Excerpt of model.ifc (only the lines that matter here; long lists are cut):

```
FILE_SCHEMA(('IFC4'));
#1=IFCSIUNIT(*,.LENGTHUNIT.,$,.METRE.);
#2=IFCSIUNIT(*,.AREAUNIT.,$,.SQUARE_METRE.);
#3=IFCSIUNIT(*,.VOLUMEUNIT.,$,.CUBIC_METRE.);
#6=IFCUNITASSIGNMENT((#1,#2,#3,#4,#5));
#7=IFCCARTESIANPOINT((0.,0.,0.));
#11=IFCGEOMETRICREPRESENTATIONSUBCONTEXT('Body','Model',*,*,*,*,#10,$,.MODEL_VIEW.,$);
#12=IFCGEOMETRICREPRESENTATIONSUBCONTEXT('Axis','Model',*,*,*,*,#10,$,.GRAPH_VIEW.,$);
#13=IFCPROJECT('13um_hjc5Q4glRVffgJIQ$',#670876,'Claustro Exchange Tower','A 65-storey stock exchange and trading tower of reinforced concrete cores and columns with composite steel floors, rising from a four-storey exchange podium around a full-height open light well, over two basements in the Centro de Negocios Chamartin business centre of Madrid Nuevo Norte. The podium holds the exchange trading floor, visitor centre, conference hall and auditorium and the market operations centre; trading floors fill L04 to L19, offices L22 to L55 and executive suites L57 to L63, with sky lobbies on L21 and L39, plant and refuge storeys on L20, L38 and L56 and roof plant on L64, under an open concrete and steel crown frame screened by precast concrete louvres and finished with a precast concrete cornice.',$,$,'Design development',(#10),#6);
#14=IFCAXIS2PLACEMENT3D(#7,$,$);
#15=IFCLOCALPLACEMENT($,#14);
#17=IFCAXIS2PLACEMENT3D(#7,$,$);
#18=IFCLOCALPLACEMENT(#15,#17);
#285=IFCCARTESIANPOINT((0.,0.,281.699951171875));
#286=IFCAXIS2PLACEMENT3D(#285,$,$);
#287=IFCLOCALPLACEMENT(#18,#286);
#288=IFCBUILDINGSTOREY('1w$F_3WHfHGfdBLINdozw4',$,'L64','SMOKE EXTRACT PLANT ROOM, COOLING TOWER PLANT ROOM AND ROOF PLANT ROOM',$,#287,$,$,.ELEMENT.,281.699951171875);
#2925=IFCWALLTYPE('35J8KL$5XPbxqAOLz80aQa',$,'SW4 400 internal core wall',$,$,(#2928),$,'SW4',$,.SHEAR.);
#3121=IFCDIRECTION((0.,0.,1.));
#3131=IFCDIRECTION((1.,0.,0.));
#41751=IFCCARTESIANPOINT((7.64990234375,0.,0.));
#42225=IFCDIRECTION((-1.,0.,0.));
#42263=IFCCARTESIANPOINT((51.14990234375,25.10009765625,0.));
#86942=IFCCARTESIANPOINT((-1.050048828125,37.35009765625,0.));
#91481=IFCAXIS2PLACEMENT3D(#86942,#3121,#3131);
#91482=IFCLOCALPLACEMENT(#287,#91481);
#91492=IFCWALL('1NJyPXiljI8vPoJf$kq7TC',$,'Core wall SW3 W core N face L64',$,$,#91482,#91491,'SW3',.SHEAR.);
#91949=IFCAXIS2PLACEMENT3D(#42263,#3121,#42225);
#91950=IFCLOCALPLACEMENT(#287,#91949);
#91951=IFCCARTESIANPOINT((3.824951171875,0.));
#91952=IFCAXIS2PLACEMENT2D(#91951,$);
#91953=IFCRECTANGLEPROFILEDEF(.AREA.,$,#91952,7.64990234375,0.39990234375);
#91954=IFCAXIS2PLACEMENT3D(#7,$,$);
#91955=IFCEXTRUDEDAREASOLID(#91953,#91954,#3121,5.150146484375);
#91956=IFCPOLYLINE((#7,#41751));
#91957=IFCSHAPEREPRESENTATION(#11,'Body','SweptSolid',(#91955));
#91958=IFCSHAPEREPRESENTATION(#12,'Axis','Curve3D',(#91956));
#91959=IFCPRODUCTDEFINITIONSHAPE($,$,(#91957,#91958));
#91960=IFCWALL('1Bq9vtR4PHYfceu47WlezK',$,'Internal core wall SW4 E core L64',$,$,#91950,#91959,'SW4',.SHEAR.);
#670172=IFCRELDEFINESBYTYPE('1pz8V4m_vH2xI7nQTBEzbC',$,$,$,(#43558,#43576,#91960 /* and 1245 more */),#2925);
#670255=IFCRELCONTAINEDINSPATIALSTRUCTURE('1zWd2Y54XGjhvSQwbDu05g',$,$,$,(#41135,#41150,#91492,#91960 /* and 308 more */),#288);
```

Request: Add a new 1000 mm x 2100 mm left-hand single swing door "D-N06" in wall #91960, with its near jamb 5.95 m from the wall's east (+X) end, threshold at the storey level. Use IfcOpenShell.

```python
import numpy as np
import ifcopenshell
import ifcopenshell.api.feature
import ifcopenshell.api.geometry
import ifcopenshell.api.root
import ifcopenshell.api.spatial
import ifcopenshell.geom
import ifcopenshell.util.element
import ifcopenshell.util.placement
import ifcopenshell.util.representation
import ifcopenshell.util.shape
import ifcopenshell.util.unit

model = ifcopenshell.open("model.ifc")
unit_scale = ifcopenshell.util.unit.calculate_unit_scale(model)
settings = ifcopenshell.geom.settings()


def volume(element):
    """Net volume in cubic metres, openings subtracted."""
    shape = ifcopenshell.geom.create_shape(settings, element)
    return ifcopenshell.util.shape.get_volume(shape.geometry)


wall = model.by_id(91960)
storey = ifcopenshell.util.element.get_container(wall, ifc_class="IfcBuildingStorey")
context = ifcopenshell.util.representation.get_context(model, "Model", "Body", "MODEL_VIEW")
before = volume(wall)

width, height, from_end, sill = 1, 2.1, 5.95, 0.0  # metres

# The wall runs along its own X axis, and the end named is its -X end.
wall_shape = ifcopenshell.geom.create_shape(settings, wall)
x, y, z = ifcopenshell.util.shape.get_vertices(wall_shape.geometry).T
start = x.min() + from_end
face, thickness = float(y.min()), float(y.max() - y.min())
wall_matrix = ifcopenshell.util.placement.get_local_placement(wall.ObjectPlacement)
level = ifcopenshell.util.placement.get_local_placement(storey.ObjectPlacement)[2, 3]


def in_wall(x, y):
    """Placement at x, y metres in the wall's axes, at sill height."""
    matrix = wall_matrix.copy()
    matrix[:, 3] = wall_matrix @ np.array([x / unit_scale, y / unit_scale, 0.0, 1.0])
    matrix[2, 3] = level + sill / unit_scale
    return matrix


# Opening: a box that overshoots both wall faces by 50 mm.
opening = ifcopenshell.api.root.create_entity(model, ifc_class="IfcOpeningElement", predefined_type="OPENING")
box = ifcopenshell.api.geometry.add_wall_representation(
    model, context=context, length=width, height=height, thickness=thickness + 0.1
)
ifcopenshell.api.geometry.assign_representation(model, product=opening, representation=box)
ifcopenshell.api.geometry.edit_object_placement(model, product=opening, matrix=in_wall(start, face - 0.05), is_si=False)
ifcopenshell.api.feature.add_feature(model, feature=opening, element=wall)

door = ifcopenshell.api.root.create_entity(model, ifc_class="IfcDoor", name="D-N06", predefined_type="DOOR")
door.OverallWidth, door.OverallHeight = width / unit_scale, height / unit_scale
door.OperationType = "SINGLE_SWING_LEFT"
body = ifcopenshell.api.geometry.add_door_representation(
    model,
    context=context,
    overall_width=door.OverallWidth,
    overall_height=door.OverallHeight,
    operation_type="SINGLE_SWING_LEFT",
    lining_properties={"LiningDepth": thickness / unit_scale, "ThresholdDepth": thickness / unit_scale},
)
ifcopenshell.api.geometry.assign_representation(model, product=door, representation=body)
ifcopenshell.api.spatial.assign_container(model, products=[door], relating_structure=storey)
ifcopenshell.api.feature.add_filling(model, opening=opening, element=door)

# The lining spans the wall, so the door starts at the wall face.
ifcopenshell.api.geometry.edit_object_placement(model, product=door, matrix=in_wall(start, face), is_si=False)

after = volume(wall)

print(f"wall volume {before:.3f} -> {after:.3f} m3")

model.write("model_updated.ifc")
```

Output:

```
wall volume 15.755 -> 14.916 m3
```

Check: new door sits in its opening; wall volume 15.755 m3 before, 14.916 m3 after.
